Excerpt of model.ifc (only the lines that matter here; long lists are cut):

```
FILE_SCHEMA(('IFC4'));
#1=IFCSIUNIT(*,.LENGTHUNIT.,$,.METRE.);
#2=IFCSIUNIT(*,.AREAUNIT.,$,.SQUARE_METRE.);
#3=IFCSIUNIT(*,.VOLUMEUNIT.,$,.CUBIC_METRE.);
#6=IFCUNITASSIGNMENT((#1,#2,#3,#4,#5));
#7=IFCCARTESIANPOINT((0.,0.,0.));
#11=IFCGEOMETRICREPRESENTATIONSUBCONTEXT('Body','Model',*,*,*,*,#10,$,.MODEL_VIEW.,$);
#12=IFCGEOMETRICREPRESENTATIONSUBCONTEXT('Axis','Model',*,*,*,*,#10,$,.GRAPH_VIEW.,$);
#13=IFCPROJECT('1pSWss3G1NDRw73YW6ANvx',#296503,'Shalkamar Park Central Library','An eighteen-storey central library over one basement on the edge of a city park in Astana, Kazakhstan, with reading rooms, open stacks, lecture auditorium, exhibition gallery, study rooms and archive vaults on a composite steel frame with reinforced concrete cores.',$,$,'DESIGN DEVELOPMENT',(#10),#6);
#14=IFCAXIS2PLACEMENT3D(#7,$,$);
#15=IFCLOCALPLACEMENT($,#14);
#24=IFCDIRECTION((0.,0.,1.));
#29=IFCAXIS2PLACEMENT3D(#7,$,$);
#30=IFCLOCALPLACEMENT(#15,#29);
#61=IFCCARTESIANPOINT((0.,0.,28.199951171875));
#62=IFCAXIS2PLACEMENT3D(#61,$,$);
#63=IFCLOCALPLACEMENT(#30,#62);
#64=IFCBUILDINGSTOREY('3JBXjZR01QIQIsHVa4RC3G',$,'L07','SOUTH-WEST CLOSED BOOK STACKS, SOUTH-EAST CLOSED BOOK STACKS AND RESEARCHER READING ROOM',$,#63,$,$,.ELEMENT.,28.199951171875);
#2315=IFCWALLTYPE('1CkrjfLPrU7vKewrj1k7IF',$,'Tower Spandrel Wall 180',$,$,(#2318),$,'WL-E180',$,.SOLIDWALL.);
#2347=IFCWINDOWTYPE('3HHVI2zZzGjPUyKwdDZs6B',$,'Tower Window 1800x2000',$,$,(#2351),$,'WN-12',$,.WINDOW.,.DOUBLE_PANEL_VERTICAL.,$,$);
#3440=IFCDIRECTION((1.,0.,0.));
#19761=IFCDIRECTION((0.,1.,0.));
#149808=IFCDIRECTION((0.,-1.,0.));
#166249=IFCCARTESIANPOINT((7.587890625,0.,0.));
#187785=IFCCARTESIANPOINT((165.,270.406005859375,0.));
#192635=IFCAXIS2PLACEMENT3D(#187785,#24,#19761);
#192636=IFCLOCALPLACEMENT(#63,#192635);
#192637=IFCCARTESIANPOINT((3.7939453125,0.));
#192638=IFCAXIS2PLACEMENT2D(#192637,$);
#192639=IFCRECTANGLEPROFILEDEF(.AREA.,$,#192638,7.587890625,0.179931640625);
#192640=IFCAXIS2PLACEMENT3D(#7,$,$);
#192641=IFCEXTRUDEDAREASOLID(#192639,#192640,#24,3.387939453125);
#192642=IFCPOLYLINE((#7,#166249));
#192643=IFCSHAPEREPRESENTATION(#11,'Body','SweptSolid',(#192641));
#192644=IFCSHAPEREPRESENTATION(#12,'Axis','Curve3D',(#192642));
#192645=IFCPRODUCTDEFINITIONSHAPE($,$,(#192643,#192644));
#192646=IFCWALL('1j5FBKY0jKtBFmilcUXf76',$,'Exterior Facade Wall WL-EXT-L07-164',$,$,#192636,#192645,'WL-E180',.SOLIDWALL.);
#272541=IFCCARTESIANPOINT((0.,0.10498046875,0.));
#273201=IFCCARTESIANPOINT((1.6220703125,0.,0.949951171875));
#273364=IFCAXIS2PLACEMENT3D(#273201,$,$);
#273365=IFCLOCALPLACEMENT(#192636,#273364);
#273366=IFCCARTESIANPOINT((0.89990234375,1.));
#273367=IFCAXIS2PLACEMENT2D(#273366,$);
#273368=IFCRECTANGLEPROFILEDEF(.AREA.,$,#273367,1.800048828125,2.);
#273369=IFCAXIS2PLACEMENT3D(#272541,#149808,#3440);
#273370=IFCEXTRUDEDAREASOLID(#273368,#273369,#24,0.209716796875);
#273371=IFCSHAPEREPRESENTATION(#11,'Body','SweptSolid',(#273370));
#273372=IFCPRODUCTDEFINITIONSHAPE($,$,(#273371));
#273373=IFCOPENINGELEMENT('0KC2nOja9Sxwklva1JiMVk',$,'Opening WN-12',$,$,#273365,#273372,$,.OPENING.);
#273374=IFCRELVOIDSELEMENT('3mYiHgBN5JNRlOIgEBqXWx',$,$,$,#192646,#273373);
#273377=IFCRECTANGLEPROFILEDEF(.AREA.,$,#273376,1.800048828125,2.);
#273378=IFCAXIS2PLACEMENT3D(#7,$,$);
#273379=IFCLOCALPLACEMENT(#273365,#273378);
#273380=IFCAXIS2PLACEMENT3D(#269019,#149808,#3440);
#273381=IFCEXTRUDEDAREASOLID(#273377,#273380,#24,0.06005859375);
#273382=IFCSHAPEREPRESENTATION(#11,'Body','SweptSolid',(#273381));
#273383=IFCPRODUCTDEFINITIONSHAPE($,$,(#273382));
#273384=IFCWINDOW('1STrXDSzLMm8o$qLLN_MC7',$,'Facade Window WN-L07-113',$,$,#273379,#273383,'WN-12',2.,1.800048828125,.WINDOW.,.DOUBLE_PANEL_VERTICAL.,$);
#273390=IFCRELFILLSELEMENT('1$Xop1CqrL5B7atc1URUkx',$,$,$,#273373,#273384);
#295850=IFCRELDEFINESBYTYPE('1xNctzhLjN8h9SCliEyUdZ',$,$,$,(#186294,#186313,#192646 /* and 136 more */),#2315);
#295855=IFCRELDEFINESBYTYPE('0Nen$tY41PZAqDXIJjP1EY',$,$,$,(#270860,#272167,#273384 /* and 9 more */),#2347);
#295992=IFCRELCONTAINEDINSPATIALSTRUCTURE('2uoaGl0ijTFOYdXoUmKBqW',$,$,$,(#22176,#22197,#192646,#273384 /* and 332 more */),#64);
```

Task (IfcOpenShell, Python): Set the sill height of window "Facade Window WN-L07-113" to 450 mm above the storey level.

```python
import numpy as np
import ifcopenshell
import ifcopenshell.api.geometry
import ifcopenshell.geom
import ifcopenshell.util.element
import ifcopenshell.util.placement
import ifcopenshell.util.shape
import ifcopenshell.util.unit

model = ifcopenshell.open("model.ifc")
unit_scale = ifcopenshell.util.unit.calculate_unit_scale(model)

window = model.by_guid("1STrXDSzLMm8o$qLLN_MC7")
opening = window.FillsVoids[0].RelatingOpeningElement
storey = ifcopenshell.util.element.get_container(window, ifc_class="IfcBuildingStorey")
level = ifcopenshell.util.placement.get_local_placement(storey.ObjectPlacement)[2, 3]

# The opening's origin need not be at the sill, so measure its lowest point.
shape = ifcopenshell.geom.create_shape(ifcopenshell.geom.settings(), opening)
bottom = ifcopenshell.util.shape.get_shape_bottom_elevation(shape, shape.geometry) / unit_scale
dz = level + 0.45 - bottom

shift = np.array([0.0, 0.0, dz])
# The window is placed relative to its opening, so it follows when the opening moves.
matrix = ifcopenshell.util.placement.get_local_placement(opening.ObjectPlacement)
matrix[:3, 3] += shift
ifcopenshell.api.geometry.edit_object_placement(
    model, product=opening, matrix=matrix, is_si=False, should_transform_children=True
)

print(f"moved by {dz * unit_scale:+.3f} m")

model.write("model_edited.ifc")
```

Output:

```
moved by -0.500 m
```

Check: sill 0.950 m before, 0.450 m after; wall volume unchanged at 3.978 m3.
